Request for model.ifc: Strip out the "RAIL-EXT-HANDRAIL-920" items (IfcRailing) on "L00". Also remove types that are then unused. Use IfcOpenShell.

First a look at what the model holds.

```python
import ifcopenshell
import ifcopenshell.util.element

model = ifcopenshell.open("model.ifc")
print(model.schema)
storey = next(s for s in model.by_type("IfcBuildingStorey") if s.Name == "L00")
railings = [e for e in ifcopenshell.util.element.get_decomposition(storey) if e.is_a("IfcRailing")]
seen = {}
for e in railings:
    element_type = ifcopenshell.util.element.get_type(e)
    name = element_type.Name if element_type not in (None, e) else None
    seen[name] = seen.get(name, 0) + 1
for name, count in sorted(seen.items(), key=str):
    print(count, "x", name)
```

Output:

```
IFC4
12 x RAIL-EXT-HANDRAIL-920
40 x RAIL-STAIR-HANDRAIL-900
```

```python
import ifcopenshell
import ifcopenshell.api.root
import ifcopenshell.util.element

model = ifcopenshell.open("model.ifc")

storey = next(s for s in model.by_type("IfcBuildingStorey") if s.Name == "L00")
railings = [e for e in ifcopenshell.util.element.get_decomposition(storey) if e.is_a("IfcRailing")]
targets = [e for e in railings if (t := ifcopenshell.util.element.get_type(e)) not in (None, e) and t.Name == "RAIL-EXT-HANDRAIL-920"]
types = {ifcopenshell.util.element.get_type(e) for e in targets} - {None, *targets}

for e in targets:
    ifcopenshell.api.root.remove_product(model, product=e)
print(len(targets), "removed")

unused = [t for t in types if not ifcopenshell.util.element.get_types(t)]
for t in unused:
    ifcopenshell.api.root.remove_product(model, product=t)
print(len(unused), "unused types removed")

model.write("model_rev.ifc")
```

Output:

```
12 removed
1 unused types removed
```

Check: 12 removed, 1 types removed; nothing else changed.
